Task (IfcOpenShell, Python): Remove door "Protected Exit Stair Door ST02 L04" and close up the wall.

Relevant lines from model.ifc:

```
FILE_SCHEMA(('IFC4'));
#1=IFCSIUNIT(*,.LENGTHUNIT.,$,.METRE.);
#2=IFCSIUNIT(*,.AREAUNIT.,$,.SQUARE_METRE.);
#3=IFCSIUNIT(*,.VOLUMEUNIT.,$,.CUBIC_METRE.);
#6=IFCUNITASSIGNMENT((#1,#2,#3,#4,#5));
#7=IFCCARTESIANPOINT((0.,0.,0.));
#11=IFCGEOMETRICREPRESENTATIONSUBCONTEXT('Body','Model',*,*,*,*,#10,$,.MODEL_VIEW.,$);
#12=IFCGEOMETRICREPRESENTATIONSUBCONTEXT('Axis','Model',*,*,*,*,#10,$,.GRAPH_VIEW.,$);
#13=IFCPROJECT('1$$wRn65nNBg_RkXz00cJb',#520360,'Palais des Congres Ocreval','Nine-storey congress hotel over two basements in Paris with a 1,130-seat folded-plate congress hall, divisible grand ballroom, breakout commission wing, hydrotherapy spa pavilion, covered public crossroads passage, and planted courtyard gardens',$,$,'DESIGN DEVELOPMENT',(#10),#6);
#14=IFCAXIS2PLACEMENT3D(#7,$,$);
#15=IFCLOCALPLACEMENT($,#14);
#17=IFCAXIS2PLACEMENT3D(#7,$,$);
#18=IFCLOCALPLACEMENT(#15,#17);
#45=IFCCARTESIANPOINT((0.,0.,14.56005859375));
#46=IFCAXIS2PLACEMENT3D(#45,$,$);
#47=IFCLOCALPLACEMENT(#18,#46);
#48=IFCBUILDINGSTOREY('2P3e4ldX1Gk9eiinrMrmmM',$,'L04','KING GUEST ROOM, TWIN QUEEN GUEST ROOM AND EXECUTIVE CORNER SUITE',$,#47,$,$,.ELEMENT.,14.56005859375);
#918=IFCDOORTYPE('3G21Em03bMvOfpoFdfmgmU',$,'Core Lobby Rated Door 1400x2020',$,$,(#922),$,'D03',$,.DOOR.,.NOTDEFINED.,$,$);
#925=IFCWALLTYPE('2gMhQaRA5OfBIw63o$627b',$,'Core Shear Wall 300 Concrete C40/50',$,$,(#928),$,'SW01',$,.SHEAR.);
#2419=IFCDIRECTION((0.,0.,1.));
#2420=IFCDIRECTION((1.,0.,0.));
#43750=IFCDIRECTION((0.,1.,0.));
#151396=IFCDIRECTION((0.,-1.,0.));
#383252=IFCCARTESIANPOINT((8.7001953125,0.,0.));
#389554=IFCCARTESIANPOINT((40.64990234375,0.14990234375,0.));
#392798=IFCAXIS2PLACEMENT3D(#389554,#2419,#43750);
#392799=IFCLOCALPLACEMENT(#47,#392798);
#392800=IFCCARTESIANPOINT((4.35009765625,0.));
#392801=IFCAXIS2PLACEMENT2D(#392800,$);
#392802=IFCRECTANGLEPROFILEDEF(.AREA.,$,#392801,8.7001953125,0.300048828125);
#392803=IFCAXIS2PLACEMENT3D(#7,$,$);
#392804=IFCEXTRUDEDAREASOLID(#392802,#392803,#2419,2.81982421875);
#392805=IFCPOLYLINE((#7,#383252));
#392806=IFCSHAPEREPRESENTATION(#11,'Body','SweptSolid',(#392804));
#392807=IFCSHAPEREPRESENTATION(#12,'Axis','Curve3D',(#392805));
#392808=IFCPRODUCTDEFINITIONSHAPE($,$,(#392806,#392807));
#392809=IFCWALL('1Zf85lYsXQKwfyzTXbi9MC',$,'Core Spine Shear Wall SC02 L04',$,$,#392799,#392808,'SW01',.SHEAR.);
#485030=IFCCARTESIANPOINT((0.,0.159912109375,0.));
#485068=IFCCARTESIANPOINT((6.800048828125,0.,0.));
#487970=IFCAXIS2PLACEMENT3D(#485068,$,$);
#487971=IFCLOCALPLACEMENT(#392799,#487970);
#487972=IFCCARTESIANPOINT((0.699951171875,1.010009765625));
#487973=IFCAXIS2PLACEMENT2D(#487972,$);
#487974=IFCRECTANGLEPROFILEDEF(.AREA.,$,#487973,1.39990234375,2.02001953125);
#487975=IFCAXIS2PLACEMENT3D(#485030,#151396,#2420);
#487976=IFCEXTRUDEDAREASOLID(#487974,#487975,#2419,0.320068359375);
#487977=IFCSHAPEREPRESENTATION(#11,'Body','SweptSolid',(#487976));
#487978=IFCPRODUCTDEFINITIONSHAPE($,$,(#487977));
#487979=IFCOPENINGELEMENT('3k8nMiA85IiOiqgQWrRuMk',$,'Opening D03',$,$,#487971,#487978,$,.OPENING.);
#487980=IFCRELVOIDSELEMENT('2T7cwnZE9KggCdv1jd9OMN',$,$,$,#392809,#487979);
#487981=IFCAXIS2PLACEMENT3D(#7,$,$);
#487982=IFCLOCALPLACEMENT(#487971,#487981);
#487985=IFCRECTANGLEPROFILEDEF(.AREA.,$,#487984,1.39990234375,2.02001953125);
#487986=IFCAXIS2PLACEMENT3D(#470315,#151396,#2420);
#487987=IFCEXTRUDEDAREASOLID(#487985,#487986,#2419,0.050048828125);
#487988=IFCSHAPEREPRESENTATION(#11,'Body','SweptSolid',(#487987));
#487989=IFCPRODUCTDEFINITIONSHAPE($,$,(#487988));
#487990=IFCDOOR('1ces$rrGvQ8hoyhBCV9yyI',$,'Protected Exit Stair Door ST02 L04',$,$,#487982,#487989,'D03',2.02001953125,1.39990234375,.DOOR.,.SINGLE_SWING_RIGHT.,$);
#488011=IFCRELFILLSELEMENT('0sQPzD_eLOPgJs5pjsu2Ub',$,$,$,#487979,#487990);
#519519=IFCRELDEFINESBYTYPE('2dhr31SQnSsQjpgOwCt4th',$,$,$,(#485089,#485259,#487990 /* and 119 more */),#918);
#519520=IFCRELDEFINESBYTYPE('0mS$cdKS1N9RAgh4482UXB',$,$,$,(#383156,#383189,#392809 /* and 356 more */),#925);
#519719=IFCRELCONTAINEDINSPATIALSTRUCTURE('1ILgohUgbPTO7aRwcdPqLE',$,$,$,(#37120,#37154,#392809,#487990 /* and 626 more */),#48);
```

```python
import ifcopenshell
import ifcopenshell.api.feature
import ifcopenshell.api.root
import ifcopenshell.geom
import ifcopenshell.util.shape

model = ifcopenshell.open("model.ifc")
settings = ifcopenshell.geom.settings()


def volume(element):
    """Net volume in cubic metres, openings subtracted."""
    shape = ifcopenshell.geom.create_shape(settings, element)
    return ifcopenshell.util.shape.get_volume(shape.geometry)


door = model.by_id(487990)
opening = door.FillsVoids[0].RelatingOpeningElement
wall = opening.VoidsElements[0].RelatingBuildingElement
before = volume(wall)

ifcopenshell.api.root.remove_product(model, product=door)
ifcopenshell.api.feature.remove_feature(model, feature=opening)

after = volume(wall)

print(f"wall volume {before:.3f} -> {after:.3f} m3")

model.write("model-out.ifc")
```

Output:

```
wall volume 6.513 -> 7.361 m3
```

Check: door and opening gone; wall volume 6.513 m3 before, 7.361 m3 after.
